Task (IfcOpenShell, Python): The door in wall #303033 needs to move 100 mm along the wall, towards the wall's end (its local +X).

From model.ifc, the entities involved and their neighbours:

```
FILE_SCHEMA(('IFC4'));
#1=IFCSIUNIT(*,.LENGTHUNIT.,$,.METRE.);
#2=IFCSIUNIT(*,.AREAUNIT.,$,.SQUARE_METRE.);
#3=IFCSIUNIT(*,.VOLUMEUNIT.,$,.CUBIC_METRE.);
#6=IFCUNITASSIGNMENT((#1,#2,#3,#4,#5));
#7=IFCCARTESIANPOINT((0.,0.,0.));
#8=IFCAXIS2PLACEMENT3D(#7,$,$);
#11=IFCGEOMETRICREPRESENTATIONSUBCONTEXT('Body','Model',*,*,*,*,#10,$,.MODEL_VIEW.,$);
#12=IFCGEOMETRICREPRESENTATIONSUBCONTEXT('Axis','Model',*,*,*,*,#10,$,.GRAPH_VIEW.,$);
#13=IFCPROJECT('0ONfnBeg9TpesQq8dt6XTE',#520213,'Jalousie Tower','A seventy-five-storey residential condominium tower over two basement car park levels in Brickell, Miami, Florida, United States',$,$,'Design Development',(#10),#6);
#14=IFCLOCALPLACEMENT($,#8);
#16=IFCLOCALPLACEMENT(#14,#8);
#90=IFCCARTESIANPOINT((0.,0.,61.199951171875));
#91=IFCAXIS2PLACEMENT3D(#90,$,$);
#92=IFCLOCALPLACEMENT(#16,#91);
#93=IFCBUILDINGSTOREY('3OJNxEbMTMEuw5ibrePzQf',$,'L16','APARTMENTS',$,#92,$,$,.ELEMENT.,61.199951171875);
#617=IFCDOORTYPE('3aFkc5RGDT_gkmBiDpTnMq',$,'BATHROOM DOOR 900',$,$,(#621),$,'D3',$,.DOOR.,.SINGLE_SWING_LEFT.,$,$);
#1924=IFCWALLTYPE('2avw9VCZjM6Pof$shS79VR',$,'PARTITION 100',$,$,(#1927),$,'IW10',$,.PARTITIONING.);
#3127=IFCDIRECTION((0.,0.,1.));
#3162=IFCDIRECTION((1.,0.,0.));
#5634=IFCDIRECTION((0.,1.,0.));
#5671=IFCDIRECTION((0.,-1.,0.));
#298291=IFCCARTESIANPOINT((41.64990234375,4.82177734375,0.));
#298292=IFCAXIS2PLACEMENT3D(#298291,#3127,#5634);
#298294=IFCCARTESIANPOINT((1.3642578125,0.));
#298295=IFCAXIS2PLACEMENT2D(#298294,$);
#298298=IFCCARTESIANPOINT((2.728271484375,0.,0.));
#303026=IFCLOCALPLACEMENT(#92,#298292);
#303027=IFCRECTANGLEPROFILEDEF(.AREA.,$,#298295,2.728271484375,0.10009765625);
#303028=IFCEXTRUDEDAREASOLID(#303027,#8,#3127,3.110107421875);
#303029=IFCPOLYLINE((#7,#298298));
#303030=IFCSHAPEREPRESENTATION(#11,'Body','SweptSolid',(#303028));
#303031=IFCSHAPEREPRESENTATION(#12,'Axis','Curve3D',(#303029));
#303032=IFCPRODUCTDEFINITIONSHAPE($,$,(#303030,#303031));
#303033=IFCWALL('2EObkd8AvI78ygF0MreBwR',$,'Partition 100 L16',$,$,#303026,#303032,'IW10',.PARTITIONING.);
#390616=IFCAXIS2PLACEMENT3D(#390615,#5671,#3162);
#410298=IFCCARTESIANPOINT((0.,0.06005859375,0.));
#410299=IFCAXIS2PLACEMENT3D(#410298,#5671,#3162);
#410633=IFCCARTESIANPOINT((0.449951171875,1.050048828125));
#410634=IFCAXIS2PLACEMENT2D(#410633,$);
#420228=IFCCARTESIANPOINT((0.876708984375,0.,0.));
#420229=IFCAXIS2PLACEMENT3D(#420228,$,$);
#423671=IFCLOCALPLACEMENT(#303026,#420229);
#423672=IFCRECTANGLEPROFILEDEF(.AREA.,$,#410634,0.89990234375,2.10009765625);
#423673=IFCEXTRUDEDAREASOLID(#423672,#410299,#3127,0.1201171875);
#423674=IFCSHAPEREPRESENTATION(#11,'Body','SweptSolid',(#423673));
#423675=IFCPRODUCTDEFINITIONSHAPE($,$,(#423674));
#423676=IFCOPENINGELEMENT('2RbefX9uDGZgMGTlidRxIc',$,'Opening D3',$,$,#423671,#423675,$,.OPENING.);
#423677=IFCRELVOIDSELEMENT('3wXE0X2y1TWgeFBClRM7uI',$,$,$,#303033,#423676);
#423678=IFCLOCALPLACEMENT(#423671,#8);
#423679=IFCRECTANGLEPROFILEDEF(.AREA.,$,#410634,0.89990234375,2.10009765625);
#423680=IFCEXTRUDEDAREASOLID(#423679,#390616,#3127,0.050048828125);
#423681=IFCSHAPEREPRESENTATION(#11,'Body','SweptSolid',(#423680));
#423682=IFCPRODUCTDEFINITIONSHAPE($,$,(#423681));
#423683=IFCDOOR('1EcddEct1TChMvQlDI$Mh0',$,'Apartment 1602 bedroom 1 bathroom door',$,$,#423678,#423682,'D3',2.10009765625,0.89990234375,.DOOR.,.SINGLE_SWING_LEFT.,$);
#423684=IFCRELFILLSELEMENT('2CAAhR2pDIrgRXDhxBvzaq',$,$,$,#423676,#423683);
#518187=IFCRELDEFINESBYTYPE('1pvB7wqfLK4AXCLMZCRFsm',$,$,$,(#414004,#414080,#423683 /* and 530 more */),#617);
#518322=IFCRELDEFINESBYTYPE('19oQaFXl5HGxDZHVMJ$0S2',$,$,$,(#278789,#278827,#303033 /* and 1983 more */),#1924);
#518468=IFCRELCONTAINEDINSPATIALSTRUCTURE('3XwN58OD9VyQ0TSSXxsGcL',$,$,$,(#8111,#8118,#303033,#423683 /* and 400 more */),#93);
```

```python
import ifcopenshell
import ifcopenshell.api.geometry
import ifcopenshell.util.placement
import ifcopenshell.util.unit

model = ifcopenshell.open("model.ifc")
unit_scale = ifcopenshell.util.unit.calculate_unit_scale(model)

door = model.by_id(423683)
opening = door.FillsVoids[0].RelatingOpeningElement
wall = opening.VoidsElements[0].RelatingBuildingElement

wall_matrix = ifcopenshell.util.placement.get_local_placement(wall.ObjectPlacement)
shift = wall_matrix[:3, 0] * 0.1 / unit_scale
before = ifcopenshell.util.placement.get_local_placement(door.ObjectPlacement)[:3, 3].copy()

# The door is placed relative to its opening, so it follows when the opening moves.
matrix = ifcopenshell.util.placement.get_local_placement(opening.ObjectPlacement)
matrix[:3, 3] += shift
ifcopenshell.api.geometry.edit_object_placement(
    model, product=opening, matrix=matrix, is_si=False, should_transform_children=True
)

after = ifcopenshell.util.placement.get_local_placement(door.ObjectPlacement)[:3, 3]
print("door moved by", (after - before).round(3) + 0.0)

model.write("model_rev.ifc")
```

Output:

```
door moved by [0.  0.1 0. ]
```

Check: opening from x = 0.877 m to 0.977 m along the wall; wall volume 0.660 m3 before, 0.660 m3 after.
